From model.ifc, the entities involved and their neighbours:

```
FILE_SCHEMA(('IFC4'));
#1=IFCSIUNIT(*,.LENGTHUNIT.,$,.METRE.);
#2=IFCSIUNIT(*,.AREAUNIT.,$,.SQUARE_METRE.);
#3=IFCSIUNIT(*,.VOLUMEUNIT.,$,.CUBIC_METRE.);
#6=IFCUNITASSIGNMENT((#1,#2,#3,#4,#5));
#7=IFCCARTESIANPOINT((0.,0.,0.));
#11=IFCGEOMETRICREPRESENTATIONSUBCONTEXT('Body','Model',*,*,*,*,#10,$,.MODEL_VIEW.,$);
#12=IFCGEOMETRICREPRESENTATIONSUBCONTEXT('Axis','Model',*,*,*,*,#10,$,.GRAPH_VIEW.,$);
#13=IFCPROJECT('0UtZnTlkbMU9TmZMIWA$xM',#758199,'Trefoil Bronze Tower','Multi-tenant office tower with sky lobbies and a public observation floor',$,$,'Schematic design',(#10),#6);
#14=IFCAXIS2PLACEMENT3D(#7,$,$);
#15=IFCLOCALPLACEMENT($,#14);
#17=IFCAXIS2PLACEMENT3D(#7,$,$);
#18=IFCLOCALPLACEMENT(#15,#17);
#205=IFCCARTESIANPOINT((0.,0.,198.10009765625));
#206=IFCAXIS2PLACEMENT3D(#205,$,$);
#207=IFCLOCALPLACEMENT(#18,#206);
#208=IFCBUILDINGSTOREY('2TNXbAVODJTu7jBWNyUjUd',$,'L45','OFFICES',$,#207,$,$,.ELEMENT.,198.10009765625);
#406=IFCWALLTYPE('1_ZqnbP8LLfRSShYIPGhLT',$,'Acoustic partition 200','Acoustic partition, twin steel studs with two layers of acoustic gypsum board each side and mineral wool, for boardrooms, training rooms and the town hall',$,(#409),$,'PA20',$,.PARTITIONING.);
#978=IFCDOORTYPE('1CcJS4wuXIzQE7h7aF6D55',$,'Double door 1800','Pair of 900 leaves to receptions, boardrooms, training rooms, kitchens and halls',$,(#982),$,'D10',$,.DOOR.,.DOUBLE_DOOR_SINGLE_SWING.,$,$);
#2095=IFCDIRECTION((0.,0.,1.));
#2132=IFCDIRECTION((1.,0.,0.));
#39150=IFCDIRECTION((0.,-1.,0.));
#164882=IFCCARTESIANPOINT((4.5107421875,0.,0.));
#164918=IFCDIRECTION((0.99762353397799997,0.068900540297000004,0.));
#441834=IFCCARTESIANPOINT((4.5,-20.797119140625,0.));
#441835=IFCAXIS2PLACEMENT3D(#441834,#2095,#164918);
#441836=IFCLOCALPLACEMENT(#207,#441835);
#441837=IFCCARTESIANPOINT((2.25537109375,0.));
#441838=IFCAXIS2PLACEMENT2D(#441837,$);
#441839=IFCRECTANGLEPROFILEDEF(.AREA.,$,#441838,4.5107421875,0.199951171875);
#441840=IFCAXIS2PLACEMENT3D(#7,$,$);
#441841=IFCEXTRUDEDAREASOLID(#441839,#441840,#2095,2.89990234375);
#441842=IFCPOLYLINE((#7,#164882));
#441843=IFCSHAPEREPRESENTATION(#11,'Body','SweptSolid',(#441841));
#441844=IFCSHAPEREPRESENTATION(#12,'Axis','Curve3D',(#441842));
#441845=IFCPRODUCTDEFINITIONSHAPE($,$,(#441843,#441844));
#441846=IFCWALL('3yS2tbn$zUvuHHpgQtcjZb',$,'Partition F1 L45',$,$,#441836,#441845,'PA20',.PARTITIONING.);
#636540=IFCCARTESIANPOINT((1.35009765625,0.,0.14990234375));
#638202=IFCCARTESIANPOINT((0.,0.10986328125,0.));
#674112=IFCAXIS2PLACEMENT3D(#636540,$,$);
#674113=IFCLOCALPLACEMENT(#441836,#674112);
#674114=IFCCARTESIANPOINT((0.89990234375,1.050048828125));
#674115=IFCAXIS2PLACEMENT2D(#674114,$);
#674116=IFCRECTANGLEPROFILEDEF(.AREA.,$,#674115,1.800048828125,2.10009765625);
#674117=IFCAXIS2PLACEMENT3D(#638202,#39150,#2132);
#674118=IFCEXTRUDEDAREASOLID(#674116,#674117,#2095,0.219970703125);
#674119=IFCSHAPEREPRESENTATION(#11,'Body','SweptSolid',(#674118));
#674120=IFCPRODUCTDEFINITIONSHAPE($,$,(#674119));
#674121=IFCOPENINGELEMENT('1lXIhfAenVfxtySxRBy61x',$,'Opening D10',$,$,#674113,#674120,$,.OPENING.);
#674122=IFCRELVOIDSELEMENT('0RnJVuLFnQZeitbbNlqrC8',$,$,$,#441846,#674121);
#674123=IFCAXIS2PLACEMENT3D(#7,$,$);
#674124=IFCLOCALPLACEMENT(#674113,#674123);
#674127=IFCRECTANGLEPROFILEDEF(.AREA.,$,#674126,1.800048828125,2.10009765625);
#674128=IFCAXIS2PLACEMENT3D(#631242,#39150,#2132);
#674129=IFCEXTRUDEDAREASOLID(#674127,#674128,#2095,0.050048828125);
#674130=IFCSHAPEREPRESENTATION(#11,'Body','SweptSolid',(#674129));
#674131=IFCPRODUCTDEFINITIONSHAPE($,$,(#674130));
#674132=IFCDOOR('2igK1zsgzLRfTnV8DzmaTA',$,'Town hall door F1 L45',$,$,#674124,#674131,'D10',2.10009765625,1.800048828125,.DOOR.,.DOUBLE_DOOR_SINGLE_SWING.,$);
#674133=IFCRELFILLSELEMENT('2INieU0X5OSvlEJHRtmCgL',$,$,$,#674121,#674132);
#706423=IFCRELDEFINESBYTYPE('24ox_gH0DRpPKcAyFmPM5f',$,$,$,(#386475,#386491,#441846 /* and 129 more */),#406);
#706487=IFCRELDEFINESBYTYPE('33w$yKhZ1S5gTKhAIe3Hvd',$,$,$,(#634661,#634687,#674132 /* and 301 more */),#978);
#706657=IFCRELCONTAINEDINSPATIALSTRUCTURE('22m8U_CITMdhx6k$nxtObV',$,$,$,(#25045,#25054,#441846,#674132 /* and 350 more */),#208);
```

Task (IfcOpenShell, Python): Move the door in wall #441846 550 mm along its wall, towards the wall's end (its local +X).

```python
import ifcopenshell
import ifcopenshell.api.geometry
import ifcopenshell.util.placement

model = ifcopenshell.open("model.ifc")

door = model.by_id(674132)
opening = door.FillsVoids[0].RelatingOpeningElement
wall = opening.VoidsElements[0].RelatingBuildingElement

wall_matrix = ifcopenshell.util.placement.get_local_placement(wall.ObjectPlacement)
shift = wall_matrix[:3, 0] * 0.55
before = ifcopenshell.util.placement.get_local_placement(door.ObjectPlacement)[:3, 3].copy()

# The door is placed relative to its opening, so it follows when the opening moves.
matrix = ifcopenshell.util.placement.get_local_placement(opening.ObjectPlacement)
matrix[:3, 3] += shift
ifcopenshell.api.geometry.edit_object_placement(
    model, product=opening, matrix=matrix, is_si=False, should_transform_children=True
)

after = ifcopenshell.util.placement.get_local_placement(door.ObjectPlacement)[:3, 3]
print("door moved by", (after - before).round(3) + 0.0)

model.write("model_v2.ifc")
```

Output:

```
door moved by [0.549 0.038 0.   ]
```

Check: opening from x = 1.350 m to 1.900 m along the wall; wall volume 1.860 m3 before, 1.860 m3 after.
